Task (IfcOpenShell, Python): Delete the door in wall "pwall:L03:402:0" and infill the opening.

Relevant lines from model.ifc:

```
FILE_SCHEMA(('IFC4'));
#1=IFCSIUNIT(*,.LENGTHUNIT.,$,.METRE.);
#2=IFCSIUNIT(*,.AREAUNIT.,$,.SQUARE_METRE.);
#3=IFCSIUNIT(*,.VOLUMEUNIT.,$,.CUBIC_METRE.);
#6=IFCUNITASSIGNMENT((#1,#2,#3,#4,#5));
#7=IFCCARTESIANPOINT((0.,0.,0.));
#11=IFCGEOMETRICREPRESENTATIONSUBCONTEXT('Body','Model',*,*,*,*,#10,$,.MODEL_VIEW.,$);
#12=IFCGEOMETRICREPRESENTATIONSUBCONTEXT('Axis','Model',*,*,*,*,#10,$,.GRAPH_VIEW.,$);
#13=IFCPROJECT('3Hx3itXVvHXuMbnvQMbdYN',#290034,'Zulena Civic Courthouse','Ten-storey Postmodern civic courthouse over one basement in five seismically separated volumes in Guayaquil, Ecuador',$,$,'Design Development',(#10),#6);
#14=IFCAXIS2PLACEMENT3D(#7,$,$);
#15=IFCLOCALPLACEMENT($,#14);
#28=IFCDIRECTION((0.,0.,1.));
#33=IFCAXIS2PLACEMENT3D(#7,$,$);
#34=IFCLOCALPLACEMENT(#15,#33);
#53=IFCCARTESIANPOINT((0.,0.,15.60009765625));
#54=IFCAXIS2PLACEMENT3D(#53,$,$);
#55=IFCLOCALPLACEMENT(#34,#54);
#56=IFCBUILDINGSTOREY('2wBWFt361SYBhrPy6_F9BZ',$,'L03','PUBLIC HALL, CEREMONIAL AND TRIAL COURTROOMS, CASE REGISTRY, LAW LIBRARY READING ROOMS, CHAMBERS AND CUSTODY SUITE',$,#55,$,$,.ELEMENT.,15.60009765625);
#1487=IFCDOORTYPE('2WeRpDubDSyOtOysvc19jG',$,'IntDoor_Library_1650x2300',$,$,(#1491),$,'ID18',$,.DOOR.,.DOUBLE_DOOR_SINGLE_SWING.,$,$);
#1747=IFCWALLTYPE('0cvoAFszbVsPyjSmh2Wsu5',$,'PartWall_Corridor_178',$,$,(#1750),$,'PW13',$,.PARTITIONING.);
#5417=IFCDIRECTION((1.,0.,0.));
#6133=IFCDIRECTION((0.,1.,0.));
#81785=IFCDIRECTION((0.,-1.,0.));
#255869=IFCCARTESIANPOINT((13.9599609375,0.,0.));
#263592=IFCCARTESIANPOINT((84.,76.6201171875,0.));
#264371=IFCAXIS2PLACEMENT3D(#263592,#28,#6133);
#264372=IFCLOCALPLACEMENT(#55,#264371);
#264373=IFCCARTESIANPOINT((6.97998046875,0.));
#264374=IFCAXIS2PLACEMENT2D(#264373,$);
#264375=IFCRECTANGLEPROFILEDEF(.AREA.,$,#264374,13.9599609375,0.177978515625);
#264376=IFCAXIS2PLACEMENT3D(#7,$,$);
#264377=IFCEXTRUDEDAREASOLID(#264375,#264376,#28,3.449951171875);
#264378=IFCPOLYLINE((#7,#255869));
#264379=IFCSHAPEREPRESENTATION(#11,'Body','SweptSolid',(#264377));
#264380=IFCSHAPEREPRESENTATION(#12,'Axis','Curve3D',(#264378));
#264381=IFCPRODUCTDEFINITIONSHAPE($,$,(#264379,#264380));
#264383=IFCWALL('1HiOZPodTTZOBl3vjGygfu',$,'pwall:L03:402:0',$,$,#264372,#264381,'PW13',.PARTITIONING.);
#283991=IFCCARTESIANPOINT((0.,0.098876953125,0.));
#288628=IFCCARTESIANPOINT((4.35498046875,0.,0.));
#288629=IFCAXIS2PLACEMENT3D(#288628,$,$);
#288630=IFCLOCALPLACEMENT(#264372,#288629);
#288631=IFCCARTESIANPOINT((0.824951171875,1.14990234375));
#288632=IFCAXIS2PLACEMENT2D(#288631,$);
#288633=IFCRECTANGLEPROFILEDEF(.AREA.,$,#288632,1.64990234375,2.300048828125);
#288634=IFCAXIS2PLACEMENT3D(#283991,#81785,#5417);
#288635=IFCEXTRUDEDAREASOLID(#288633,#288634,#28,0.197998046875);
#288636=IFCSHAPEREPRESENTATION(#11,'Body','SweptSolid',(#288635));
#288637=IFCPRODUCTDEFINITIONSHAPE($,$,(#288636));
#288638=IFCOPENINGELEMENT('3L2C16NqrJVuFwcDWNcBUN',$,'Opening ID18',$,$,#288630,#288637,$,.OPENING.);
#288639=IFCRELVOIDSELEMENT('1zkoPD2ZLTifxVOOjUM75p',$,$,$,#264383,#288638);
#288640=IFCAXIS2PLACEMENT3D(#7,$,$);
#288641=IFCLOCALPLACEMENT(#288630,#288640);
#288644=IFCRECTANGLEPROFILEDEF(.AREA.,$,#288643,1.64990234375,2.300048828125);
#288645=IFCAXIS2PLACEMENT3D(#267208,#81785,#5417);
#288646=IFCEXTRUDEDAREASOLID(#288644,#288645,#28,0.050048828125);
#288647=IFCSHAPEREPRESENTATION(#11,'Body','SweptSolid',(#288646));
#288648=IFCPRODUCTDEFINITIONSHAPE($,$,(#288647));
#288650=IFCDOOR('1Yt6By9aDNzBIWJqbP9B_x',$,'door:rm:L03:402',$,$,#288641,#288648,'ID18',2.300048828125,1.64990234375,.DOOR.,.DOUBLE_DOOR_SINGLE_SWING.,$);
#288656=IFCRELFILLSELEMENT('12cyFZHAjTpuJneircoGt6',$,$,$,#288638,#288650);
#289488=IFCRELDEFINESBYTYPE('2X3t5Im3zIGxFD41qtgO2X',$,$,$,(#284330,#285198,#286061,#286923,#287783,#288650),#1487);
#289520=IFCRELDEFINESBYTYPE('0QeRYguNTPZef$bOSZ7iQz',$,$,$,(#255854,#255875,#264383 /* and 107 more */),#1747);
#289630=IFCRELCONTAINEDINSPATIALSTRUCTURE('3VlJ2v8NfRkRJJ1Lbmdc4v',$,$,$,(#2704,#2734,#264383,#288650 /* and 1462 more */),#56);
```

```python
import ifcopenshell
import ifcopenshell.api.feature
import ifcopenshell.api.root
import ifcopenshell.geom
import ifcopenshell.util.shape

model = ifcopenshell.open("model.ifc")
settings = ifcopenshell.geom.settings()


def volume(element):
    """Net volume in cubic metres, openings subtracted."""
    shape = ifcopenshell.geom.create_shape(settings, element)
    return ifcopenshell.util.shape.get_volume(shape.geometry)


door = model.by_id(288650)
opening = door.FillsVoids[0].RelatingOpeningElement
wall = opening.VoidsElements[0].RelatingBuildingElement
before = volume(wall)

ifcopenshell.api.root.remove_product(model, product=door)
ifcopenshell.api.feature.remove_feature(model, feature=opening)

after = volume(wall)

print(f"wall volume {before:.3f} -> {after:.3f} m3")

model.write("model_v2.ifc")
```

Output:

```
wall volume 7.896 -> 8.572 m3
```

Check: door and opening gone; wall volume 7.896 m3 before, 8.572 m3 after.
